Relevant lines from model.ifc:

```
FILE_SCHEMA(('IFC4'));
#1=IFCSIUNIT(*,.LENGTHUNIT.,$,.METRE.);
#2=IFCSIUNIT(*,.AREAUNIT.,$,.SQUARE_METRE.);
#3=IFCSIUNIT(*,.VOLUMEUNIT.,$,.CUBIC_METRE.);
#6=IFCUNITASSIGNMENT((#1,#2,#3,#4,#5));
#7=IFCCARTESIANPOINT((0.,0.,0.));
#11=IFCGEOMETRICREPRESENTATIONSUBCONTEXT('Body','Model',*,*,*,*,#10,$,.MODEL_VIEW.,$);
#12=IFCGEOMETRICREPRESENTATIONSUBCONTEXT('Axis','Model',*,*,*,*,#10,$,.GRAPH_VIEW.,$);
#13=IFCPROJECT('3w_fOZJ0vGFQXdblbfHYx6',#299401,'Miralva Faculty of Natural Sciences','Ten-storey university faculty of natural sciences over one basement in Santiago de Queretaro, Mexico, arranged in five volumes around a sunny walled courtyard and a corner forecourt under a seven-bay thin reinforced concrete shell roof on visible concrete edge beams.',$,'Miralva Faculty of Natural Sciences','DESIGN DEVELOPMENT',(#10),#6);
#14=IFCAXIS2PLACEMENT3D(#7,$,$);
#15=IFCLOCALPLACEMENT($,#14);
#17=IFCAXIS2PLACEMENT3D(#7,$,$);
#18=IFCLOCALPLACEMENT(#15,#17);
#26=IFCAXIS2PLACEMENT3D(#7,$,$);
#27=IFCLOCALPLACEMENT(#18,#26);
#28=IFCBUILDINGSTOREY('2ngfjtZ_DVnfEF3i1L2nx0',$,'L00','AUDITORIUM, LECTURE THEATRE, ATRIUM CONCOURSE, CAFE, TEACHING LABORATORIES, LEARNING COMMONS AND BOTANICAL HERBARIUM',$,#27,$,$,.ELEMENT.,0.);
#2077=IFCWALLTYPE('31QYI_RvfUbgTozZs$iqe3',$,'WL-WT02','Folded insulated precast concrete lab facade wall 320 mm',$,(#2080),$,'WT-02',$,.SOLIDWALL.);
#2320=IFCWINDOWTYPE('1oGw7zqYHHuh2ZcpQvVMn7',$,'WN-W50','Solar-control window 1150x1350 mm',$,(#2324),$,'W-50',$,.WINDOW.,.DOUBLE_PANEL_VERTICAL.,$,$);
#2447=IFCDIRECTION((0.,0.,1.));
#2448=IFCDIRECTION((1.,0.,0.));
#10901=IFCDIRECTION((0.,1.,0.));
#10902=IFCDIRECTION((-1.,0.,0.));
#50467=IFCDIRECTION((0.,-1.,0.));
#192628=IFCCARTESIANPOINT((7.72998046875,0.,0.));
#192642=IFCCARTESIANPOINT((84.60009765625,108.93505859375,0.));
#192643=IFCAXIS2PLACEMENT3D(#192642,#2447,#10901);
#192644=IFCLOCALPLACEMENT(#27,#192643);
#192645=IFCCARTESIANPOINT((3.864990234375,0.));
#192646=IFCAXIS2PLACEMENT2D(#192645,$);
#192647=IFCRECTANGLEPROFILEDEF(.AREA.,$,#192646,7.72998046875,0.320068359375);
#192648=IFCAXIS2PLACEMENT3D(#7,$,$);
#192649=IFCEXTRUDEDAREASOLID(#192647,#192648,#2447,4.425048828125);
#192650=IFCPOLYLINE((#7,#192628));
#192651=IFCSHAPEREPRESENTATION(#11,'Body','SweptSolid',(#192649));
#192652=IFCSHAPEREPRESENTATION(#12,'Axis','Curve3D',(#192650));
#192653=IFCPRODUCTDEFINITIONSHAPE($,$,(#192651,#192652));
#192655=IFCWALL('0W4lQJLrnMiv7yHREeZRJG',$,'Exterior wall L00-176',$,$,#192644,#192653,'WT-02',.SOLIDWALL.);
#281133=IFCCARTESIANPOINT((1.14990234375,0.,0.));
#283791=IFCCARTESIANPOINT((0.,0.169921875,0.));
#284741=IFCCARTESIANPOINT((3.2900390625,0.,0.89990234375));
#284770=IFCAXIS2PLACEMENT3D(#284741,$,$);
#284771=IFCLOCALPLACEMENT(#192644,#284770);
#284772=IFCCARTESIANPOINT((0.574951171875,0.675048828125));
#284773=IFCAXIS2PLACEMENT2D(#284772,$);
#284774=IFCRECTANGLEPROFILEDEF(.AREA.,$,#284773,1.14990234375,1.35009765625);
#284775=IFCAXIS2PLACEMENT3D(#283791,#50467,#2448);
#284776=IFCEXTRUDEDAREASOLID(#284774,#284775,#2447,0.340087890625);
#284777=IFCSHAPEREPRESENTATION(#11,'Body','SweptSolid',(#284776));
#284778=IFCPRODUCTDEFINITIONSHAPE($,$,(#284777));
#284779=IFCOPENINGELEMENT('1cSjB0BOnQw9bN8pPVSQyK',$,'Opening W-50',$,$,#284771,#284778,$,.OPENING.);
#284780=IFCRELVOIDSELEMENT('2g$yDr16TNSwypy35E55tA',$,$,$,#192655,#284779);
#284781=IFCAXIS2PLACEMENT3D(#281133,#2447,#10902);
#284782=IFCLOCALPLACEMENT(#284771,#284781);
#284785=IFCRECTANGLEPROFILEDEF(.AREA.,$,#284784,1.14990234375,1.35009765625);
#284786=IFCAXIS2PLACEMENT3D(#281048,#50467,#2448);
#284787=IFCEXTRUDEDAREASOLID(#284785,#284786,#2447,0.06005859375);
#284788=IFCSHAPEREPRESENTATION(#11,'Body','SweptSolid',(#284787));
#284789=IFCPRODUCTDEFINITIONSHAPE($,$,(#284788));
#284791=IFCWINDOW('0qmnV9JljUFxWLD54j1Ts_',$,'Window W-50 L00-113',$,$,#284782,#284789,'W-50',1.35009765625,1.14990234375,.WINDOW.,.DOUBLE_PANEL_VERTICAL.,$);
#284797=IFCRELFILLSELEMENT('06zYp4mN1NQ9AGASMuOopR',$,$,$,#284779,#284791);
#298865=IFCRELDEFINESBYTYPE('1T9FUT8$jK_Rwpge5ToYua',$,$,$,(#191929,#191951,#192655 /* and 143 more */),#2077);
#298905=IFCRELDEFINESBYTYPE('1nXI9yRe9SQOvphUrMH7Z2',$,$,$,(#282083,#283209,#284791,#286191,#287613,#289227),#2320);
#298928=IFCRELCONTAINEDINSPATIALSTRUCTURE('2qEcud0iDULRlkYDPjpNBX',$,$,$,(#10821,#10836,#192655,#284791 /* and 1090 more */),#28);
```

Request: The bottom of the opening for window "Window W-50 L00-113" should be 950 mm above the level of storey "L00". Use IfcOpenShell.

```python
import numpy as np
import ifcopenshell
import ifcopenshell.api.geometry
import ifcopenshell.geom
import ifcopenshell.util.element
import ifcopenshell.util.placement
import ifcopenshell.util.shape
import ifcopenshell.util.unit

model = ifcopenshell.open("model.ifc")
unit_scale = ifcopenshell.util.unit.calculate_unit_scale(model)

window = model.by_guid("0qmnV9JljUFxWLD54j1Ts_")
opening = window.FillsVoids[0].RelatingOpeningElement
storey = ifcopenshell.util.element.get_container(window, ifc_class="IfcBuildingStorey")
level = ifcopenshell.util.placement.get_local_placement(storey.ObjectPlacement)[2, 3]

# The opening's origin need not be at the sill, so measure its lowest point.
shape = ifcopenshell.geom.create_shape(ifcopenshell.geom.settings(), opening)
bottom = ifcopenshell.util.shape.get_shape_bottom_elevation(shape, shape.geometry) / unit_scale
dz = level + 0.95 / unit_scale - bottom

shift = np.array([0.0, 0.0, dz])
# The window is placed relative to its opening, so it follows when the opening moves.
matrix = ifcopenshell.util.placement.get_local_placement(opening.ObjectPlacement)
matrix[:3, 3] += shift
ifcopenshell.api.geometry.edit_object_placement(
    model, product=opening, matrix=matrix, is_si=False, should_transform_children=True
)

print(f"moved by {dz * unit_scale:+.3f} m")

model.write("model_rev.ifc")
```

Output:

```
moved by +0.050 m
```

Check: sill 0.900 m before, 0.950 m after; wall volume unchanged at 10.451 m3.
